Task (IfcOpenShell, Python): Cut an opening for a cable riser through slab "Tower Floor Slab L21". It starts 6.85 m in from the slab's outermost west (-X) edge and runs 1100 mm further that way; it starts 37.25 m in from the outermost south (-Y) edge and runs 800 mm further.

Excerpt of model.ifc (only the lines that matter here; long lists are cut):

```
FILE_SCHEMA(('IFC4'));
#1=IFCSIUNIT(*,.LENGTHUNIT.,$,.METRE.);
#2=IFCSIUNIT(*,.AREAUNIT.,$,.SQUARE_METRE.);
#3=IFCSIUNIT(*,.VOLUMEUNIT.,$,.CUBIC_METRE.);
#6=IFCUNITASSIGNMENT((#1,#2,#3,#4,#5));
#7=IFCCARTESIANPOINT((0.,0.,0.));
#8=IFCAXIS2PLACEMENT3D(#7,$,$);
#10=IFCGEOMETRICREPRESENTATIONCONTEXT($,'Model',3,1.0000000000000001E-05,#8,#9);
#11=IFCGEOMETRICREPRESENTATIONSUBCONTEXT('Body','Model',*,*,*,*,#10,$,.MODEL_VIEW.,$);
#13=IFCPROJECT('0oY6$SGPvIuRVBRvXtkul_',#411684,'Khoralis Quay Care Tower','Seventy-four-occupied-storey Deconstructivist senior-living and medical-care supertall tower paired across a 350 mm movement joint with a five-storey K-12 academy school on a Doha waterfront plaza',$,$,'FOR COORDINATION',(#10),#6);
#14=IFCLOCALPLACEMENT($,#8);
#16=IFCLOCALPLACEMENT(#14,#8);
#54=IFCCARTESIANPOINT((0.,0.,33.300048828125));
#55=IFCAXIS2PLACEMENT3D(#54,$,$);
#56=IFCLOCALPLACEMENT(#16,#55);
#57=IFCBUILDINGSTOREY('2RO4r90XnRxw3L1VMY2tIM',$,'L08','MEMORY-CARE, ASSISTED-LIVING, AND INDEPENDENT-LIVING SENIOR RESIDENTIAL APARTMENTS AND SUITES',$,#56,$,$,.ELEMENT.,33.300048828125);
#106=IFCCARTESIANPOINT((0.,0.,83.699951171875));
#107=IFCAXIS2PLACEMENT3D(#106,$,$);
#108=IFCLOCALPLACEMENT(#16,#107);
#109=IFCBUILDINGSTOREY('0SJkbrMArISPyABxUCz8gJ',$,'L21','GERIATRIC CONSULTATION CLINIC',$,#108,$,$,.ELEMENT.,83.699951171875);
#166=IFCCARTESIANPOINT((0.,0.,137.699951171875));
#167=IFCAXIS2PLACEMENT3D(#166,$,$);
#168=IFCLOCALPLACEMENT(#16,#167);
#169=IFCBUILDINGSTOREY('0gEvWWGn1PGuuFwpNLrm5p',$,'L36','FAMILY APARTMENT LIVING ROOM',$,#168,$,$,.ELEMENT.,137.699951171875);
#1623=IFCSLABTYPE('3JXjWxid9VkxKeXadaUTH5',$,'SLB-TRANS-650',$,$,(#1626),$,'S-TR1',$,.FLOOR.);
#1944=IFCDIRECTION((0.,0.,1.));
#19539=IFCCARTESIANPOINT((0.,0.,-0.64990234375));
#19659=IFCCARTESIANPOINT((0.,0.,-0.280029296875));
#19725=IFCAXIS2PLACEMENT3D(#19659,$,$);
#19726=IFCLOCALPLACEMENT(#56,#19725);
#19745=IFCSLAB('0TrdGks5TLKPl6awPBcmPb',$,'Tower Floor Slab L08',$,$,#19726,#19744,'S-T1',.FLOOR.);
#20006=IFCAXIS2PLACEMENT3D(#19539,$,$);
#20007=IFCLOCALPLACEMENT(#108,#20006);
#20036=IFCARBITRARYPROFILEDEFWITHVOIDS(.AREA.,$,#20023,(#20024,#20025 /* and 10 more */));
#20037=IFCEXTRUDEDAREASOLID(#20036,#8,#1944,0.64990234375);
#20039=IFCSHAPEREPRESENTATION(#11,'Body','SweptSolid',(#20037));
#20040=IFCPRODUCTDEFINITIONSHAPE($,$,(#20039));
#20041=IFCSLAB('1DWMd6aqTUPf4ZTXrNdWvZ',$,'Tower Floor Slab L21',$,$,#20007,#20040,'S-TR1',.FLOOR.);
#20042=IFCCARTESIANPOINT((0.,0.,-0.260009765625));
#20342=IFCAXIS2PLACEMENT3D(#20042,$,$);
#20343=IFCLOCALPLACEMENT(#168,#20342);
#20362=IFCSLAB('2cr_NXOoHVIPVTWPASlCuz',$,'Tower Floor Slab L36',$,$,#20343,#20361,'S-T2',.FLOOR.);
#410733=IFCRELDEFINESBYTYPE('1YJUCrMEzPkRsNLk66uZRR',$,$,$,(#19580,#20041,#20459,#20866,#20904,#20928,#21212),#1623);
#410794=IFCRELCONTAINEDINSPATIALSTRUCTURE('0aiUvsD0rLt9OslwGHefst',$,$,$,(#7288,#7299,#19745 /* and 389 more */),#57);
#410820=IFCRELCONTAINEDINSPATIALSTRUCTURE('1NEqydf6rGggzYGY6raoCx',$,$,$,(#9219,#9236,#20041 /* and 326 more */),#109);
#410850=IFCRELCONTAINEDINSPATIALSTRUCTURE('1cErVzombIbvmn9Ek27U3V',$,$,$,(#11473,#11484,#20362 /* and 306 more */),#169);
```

```python
import numpy as np
import ifcopenshell
import ifcopenshell.api.feature
import ifcopenshell.api.geometry
import ifcopenshell.api.root
import ifcopenshell.geom
import ifcopenshell.util.placement
import ifcopenshell.util.representation
import ifcopenshell.util.shape
import ifcopenshell.util.unit

model = ifcopenshell.open("model.ifc")
unit_scale = ifcopenshell.util.unit.calculate_unit_scale(model)
settings = ifcopenshell.geom.settings()


def volume(element):
    """Net volume in cubic metres, openings subtracted."""
    shape = ifcopenshell.geom.create_shape(settings, element)
    return ifcopenshell.util.shape.get_volume(shape.geometry)


slab = model.by_guid("1DWMd6aqTUPf4ZTXrNdWvZ")
before = volume(slab)

# Extent in the slab's own axes, in metres. The edges named are its -X and -Y sides.
slab_shape = ifcopenshell.geom.create_shape(settings, slab)
vertices = ifcopenshell.util.shape.get_vertices(slab_shape.geometry)
x_min, y_min, bottom = vertices.min(axis=0)
top = vertices[:, 2].max()

opening = ifcopenshell.api.root.create_entity(model, ifc_class="IfcOpeningElement", name="Cable riser opening", predefined_type="OPENING")
context = ifcopenshell.util.representation.get_context(model, "Model", "Body", "MODEL_VIEW")
width, depth = 1.1, 0.8
outline = [(0.0, 0.0), (width, 0.0), (width, depth), (0.0, depth), (0.0, 0.0)]
# Overshoot both faces by 50 mm so the cut is clean.
shape = ifcopenshell.api.geometry.add_slab_representation(
    model, context=context, depth=top - bottom + 0.1, polyline=outline
)
ifcopenshell.api.geometry.assign_representation(model, product=opening, representation=shape)

matrix = ifcopenshell.util.placement.get_local_placement(slab.ObjectPlacement)
matrix[:, 3] = matrix @ np.append(np.array([x_min + 6.85, y_min + 37.25, bottom - 0.05]) / unit_scale, 1.0)
ifcopenshell.api.geometry.edit_object_placement(model, product=opening, matrix=matrix, is_si=False)
ifcopenshell.api.feature.add_feature(model, feature=opening, element=slab)

after = volume(slab)

print(f"slab volume {before:.3f} -> {after:.3f} m3")

model.write("model-out.ifc")
```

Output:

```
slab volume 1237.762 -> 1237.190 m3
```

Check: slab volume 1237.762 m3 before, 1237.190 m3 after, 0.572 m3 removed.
